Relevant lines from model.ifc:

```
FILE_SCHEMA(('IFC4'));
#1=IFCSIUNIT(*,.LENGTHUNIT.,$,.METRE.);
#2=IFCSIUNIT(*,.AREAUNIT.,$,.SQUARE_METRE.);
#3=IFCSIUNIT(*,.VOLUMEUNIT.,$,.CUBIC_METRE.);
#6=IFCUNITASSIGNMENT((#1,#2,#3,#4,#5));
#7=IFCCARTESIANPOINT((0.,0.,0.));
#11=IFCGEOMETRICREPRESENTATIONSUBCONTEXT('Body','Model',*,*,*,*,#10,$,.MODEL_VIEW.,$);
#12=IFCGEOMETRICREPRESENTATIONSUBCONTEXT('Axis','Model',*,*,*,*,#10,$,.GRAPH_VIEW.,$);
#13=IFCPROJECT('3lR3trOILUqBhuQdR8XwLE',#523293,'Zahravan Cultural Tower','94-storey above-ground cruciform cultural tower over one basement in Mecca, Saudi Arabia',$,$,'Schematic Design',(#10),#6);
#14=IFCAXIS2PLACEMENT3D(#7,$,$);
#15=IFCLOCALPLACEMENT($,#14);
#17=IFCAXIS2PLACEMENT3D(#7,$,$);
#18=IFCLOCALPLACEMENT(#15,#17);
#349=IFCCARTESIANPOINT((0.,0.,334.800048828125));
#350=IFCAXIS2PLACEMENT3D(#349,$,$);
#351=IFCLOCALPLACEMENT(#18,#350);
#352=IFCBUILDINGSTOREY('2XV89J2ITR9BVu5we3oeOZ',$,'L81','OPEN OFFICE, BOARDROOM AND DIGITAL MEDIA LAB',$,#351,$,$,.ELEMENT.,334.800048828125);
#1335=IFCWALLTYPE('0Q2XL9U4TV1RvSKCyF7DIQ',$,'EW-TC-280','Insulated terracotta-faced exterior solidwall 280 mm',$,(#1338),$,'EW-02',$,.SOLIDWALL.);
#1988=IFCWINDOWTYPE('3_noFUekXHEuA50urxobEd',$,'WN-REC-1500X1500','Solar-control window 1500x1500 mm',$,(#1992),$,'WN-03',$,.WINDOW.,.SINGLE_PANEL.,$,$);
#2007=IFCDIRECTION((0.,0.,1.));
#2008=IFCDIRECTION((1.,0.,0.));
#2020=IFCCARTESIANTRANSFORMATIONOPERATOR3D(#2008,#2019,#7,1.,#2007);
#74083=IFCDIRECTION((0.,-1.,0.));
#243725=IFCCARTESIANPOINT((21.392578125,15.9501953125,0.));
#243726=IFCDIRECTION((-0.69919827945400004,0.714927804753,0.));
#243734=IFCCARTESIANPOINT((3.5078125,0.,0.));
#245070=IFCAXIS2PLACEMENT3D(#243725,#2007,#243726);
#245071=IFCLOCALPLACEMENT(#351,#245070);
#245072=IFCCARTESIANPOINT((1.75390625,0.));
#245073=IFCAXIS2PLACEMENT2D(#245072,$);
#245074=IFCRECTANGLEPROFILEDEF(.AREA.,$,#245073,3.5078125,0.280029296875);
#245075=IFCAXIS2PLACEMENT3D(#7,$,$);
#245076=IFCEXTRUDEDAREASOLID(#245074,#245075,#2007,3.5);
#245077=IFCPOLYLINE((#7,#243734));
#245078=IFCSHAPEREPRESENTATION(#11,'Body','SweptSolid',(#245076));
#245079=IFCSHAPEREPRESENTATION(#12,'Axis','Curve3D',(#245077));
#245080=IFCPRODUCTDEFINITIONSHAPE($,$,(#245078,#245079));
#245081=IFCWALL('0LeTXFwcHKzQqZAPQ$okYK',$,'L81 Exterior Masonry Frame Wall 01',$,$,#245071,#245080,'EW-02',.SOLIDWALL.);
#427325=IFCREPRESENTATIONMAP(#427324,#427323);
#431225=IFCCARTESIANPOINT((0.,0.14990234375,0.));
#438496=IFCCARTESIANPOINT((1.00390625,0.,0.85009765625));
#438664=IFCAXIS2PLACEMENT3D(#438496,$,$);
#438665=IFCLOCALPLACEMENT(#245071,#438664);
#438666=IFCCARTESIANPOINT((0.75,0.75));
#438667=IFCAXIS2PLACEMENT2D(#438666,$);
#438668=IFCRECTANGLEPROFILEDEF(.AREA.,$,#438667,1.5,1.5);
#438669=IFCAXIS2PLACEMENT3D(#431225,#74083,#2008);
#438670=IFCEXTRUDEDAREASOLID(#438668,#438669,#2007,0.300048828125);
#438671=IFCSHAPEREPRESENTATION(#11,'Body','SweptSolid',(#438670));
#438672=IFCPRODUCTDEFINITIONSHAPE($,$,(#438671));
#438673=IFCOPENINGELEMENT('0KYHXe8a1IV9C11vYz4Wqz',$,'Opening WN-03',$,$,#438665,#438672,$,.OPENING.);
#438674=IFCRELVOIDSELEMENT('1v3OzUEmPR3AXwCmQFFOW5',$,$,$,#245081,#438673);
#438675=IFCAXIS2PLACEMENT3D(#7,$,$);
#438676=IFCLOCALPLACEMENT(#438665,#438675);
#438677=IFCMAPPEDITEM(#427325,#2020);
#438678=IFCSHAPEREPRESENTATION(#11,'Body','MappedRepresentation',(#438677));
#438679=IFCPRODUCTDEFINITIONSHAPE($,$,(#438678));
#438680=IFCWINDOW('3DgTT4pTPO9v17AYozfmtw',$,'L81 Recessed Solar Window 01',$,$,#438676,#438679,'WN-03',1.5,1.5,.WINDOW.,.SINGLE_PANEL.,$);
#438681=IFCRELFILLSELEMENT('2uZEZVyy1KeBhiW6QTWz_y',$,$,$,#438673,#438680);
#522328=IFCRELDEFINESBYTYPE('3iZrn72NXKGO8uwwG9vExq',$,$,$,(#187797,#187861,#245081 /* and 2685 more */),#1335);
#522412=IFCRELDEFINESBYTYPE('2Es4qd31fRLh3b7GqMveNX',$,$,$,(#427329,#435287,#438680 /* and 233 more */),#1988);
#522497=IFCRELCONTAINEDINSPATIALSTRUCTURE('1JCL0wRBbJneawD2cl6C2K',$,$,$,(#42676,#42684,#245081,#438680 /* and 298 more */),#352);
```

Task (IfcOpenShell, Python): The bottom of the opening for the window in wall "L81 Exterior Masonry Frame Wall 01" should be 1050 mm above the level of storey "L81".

```python
import numpy as np
import ifcopenshell
import ifcopenshell.api.geometry
import ifcopenshell.geom
import ifcopenshell.util.element
import ifcopenshell.util.placement
import ifcopenshell.util.shape
import ifcopenshell.util.unit

model = ifcopenshell.open("model.ifc")
unit_scale = ifcopenshell.util.unit.calculate_unit_scale(model)

window = model.by_id(438680)
opening = window.FillsVoids[0].RelatingOpeningElement
storey = ifcopenshell.util.element.get_container(window, ifc_class="IfcBuildingStorey")
level = ifcopenshell.util.placement.get_local_placement(storey.ObjectPlacement)[2, 3]

# The opening's origin need not be at the sill, so measure its lowest point.
shape = ifcopenshell.geom.create_shape(ifcopenshell.geom.settings(), opening)
bottom = ifcopenshell.util.shape.get_shape_bottom_elevation(shape, shape.geometry) / unit_scale
dz = level + 1.05 - bottom

shift = np.array([0.0, 0.0, dz])
# The window is placed relative to its opening, so it follows when the opening moves.
matrix = ifcopenshell.util.placement.get_local_placement(opening.ObjectPlacement)
matrix[:3, 3] += shift
ifcopenshell.api.geometry.edit_object_placement(
    model, product=opening, matrix=matrix, is_si=False, should_transform_children=True
)

print(f"moved by {dz * unit_scale:+.3f} m")

model.write("model_v2.ifc")
```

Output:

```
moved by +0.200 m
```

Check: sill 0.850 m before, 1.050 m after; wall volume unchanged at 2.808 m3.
